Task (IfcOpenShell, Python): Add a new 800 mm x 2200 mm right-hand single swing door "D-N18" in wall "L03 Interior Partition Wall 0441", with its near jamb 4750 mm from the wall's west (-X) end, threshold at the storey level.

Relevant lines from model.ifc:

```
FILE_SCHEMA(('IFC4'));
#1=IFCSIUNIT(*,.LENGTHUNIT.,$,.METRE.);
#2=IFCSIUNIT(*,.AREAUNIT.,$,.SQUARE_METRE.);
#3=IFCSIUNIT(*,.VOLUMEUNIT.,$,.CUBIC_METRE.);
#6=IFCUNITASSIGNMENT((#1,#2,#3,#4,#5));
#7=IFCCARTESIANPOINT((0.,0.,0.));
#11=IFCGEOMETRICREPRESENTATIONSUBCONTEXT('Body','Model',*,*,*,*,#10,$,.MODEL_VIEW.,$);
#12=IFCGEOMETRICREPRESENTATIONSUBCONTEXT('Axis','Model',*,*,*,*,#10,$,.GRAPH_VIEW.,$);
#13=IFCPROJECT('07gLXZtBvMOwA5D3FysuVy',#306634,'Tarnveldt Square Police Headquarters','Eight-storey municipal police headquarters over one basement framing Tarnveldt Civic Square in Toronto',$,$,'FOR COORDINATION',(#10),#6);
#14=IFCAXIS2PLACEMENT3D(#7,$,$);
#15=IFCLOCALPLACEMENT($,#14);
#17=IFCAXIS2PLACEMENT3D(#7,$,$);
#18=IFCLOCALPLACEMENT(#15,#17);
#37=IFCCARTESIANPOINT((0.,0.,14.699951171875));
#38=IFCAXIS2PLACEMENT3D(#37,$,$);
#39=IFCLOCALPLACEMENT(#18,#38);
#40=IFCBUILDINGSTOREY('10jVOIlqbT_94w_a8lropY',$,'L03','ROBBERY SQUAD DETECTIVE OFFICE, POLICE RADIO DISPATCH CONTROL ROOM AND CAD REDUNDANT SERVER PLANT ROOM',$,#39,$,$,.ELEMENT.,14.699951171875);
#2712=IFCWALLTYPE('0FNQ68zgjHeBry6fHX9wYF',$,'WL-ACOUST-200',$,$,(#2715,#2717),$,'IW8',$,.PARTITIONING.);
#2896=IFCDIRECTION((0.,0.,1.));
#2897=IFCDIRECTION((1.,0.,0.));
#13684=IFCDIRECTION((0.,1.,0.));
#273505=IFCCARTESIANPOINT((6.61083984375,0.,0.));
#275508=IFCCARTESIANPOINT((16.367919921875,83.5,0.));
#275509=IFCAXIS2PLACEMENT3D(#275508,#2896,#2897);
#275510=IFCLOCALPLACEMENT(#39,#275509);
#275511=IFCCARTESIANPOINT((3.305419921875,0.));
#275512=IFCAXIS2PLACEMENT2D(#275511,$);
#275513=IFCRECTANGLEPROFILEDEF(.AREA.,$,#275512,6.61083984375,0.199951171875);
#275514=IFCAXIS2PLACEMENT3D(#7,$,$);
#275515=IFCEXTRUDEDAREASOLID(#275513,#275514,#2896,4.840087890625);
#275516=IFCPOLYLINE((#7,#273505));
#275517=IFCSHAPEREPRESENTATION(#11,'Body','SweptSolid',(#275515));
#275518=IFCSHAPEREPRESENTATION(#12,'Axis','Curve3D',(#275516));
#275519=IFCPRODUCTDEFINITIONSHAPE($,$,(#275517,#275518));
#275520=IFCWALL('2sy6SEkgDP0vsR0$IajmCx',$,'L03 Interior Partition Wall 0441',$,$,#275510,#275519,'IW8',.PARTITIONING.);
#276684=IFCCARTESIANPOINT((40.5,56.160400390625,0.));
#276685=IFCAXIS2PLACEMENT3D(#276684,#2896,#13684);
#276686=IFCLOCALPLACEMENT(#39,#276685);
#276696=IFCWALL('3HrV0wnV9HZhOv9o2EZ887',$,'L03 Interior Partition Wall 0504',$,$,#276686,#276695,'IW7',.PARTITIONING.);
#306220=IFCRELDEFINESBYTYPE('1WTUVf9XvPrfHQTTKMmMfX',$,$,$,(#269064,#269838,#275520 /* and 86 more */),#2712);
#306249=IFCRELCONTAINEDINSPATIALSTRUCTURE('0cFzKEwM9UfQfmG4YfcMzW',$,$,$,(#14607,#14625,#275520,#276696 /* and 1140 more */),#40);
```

```python
import numpy as np
import ifcopenshell
import ifcopenshell.api.feature
import ifcopenshell.api.geometry
import ifcopenshell.api.root
import ifcopenshell.api.spatial
import ifcopenshell.geom
import ifcopenshell.util.element
import ifcopenshell.util.placement
import ifcopenshell.util.representation
import ifcopenshell.util.shape
import ifcopenshell.util.unit

model = ifcopenshell.open("model.ifc")
unit_scale = ifcopenshell.util.unit.calculate_unit_scale(model)
settings = ifcopenshell.geom.settings()


def volume(element):
    """Net volume in cubic metres, openings subtracted."""
    shape = ifcopenshell.geom.create_shape(settings, element)
    return ifcopenshell.util.shape.get_volume(shape.geometry)


wall = model.by_guid("2sy6SEkgDP0vsR0$IajmCx")
storey = ifcopenshell.util.element.get_container(wall, ifc_class="IfcBuildingStorey")
context = ifcopenshell.util.representation.get_context(model, "Model", "Body", "MODEL_VIEW")
before = volume(wall)

width, height, from_end, sill = 0.8, 2.2, 4.75, 0.0  # metres

# The wall runs along its own X axis, and the end named is its -X end.
wall_shape = ifcopenshell.geom.create_shape(settings, wall)
x, y, z = ifcopenshell.util.shape.get_vertices(wall_shape.geometry).T
start = x.min() + from_end
face, thickness = float(y.min()), float(y.max() - y.min())
wall_matrix = ifcopenshell.util.placement.get_local_placement(wall.ObjectPlacement)
level = ifcopenshell.util.placement.get_local_placement(storey.ObjectPlacement)[2, 3]


def in_wall(x, y):
    """Placement at x, y metres in the wall's axes, at sill height."""
    matrix = wall_matrix.copy()
    matrix[:, 3] = wall_matrix @ np.array([x / unit_scale, y / unit_scale, 0.0, 1.0])
    matrix[2, 3] = level + sill / unit_scale
    return matrix


# Opening: a box that overshoots both wall faces by 50 mm.
opening = ifcopenshell.api.root.create_entity(model, ifc_class="IfcOpeningElement", predefined_type="OPENING")
box = ifcopenshell.api.geometry.add_wall_representation(
    model, context=context, length=width, height=height, thickness=thickness + 0.1
)
ifcopenshell.api.geometry.assign_representation(model, product=opening, representation=box)
ifcopenshell.api.geometry.edit_object_placement(model, product=opening, matrix=in_wall(start, face - 0.05), is_si=False)
ifcopenshell.api.feature.add_feature(model, feature=opening, element=wall)

door = ifcopenshell.api.root.create_entity(model, ifc_class="IfcDoor", name="D-N18", predefined_type="DOOR")
door.OverallWidth, door.OverallHeight = width / unit_scale, height / unit_scale
door.OperationType = "SINGLE_SWING_RIGHT"
body = ifcopenshell.api.geometry.add_door_representation(
    model,
    context=context,
    overall_width=door.OverallWidth,
    overall_height=door.OverallHeight,
    operation_type="SINGLE_SWING_RIGHT",
    lining_properties={"LiningDepth": thickness / unit_scale, "ThresholdDepth": thickness / unit_scale},
)
ifcopenshell.api.geometry.assign_representation(model, product=door, representation=body)
ifcopenshell.api.spatial.assign_container(model, products=[door], relating_structure=storey)
ifcopenshell.api.feature.add_filling(model, opening=opening, element=door)

# The lining spans the wall, so the door starts at the wall face.
ifcopenshell.api.geometry.edit_object_placement(model, product=door, matrix=in_wall(start, face), is_si=False)

after = volume(wall)

print(f"wall volume {before:.3f} -> {after:.3f} m3")

model.write("model_rev.ifc")
```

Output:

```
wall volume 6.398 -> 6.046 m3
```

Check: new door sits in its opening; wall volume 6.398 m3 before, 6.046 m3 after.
